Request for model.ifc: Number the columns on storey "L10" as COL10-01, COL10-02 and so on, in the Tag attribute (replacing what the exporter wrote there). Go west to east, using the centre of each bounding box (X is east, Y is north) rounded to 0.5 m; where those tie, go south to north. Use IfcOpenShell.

First a look at what the model holds.

```python
import ifcopenshell
import ifcopenshell.util.element
import ifcopenshell.util.placement

model = ifcopenshell.open("model.ifc")
print(model.schema)
storey = next(s for s in model.by_type("IfcBuildingStorey") if s.Name == "L10")
columns = [e for e in ifcopenshell.util.element.get_decomposition(storey) if e.is_a("IfcColumn")]
for e in sorted(columns, key=lambda e: e.id()):
    origin = ifcopenshell.util.placement.get_local_placement(e.ObjectPlacement)[:3, 3]
    print(e.id(), e.Tag, e.Name, origin.round(2) + 0.0, sep=" | ")
```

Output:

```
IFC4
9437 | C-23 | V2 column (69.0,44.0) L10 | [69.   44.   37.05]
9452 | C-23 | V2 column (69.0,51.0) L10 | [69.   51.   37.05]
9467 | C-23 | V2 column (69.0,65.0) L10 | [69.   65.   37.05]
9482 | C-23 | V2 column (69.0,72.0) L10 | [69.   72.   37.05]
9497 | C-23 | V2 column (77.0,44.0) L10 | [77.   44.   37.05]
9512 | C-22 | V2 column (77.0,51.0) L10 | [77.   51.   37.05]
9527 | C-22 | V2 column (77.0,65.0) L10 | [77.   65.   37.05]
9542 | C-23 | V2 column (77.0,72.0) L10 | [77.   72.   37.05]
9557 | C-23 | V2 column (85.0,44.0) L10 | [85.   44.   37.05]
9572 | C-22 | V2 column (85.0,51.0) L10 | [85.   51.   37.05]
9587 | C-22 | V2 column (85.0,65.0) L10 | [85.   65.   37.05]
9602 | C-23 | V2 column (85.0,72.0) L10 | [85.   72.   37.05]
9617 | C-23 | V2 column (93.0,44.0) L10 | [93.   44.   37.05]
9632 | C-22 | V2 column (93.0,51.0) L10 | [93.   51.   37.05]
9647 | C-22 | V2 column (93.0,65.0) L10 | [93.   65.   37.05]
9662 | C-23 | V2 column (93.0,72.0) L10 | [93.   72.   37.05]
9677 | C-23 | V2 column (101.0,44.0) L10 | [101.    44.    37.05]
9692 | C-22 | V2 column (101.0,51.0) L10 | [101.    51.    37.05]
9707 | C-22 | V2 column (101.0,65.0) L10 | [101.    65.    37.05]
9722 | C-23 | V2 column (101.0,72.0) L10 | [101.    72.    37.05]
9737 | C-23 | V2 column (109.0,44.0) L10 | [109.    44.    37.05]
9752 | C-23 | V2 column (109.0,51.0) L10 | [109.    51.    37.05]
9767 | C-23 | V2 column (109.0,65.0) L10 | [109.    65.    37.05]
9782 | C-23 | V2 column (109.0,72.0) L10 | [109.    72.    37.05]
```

```python
import ifcopenshell
import ifcopenshell.geom
import ifcopenshell.util.element
import ifcopenshell.util.shape

model = ifcopenshell.open("model.ifc")
settings = ifcopenshell.geom.settings()
settings.set("use-world-coords", True)


def centre(element):
    shape = ifcopenshell.geom.create_shape(settings, element)
    return ifcopenshell.util.shape.get_bbox_centroid(shape.geometry)


storey = next(s for s in model.by_type("IfcBuildingStorey") if s.Name == "L10")
columns = [e for e in ifcopenshell.util.element.get_decomposition(storey) if e.is_a("IfcColumn")]

# Insertion points can sit at a corner or the storey origin, so sort by the geometry (in metres).
centres = {e: centre(e) for e in columns}
columns.sort(key=lambda e: (round(centres[e][0] / 0.5), centres[e][1]))

for i, e in enumerate(columns, start=1):
    number = f"COL10-{i:02d}"
    e.Tag = number
    print(e.id(), number)

model.write("model-out.ifc")
```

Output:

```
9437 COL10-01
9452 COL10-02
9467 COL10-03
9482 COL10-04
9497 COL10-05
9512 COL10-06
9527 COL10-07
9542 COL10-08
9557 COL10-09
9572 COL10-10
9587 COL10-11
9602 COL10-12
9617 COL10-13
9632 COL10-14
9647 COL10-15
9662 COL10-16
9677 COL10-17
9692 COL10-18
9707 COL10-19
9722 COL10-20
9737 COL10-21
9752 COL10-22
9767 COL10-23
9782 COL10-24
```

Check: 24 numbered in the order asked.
